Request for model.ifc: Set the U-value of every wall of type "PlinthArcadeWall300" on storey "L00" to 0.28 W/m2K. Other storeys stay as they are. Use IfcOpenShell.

First a look at what the model holds.

```python
import ifcopenshell
import ifcopenshell.util.element

model = ifcopenshell.open("model.ifc")
print(model.schema)
storey = next(s for s in model.by_type("IfcBuildingStorey") if s.Name == "L00")
walls = [e for e in ifcopenshell.util.element.get_decomposition(storey) if e.is_a("IfcWall")]
seen = {}
for e in walls:
    element_type = ifcopenshell.util.element.get_type(e)
    key = (element_type.Name if element_type != e and element_type else None, ifcopenshell.util.element.get_pset(e, "Pset_WallCommon", "ThermalTransmittance"))
    seen[key] = seen.get(key, 0) + 1
for (name, value), count in sorted(seen.items(), key=str):
    print(count, "x", name, "|", value)
```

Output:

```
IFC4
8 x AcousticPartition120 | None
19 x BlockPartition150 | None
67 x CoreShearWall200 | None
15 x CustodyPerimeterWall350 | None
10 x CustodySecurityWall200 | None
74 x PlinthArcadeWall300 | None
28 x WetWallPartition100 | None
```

```python
import ifcopenshell
import ifcopenshell.api.pset
import ifcopenshell.util.element

model = ifcopenshell.open("model.ifc")

storey = next(s for s in model.by_type("IfcBuildingStorey") if s.Name == "L00")
walls = [e for e in ifcopenshell.util.element.get_decomposition(storey) if e.is_a("IfcWall")]

count = 0
for e in walls:
    element_type = ifcopenshell.util.element.get_type(e)
    if element_type in (None, e) or element_type.Name != "PlinthArcadeWall300":
        continue
    # add_pset returns the element's existing set when there is one.
    pset = ifcopenshell.api.pset.add_pset(model, product=e, name="Pset_WallCommon")
    ifcopenshell.api.pset.edit_pset(model, pset=pset, properties={"ThermalTransmittance": 0.28})
    count += 1

print(count, "walls updated")

model.write("model_rev.ifc")
```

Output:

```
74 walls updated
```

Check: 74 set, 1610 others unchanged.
